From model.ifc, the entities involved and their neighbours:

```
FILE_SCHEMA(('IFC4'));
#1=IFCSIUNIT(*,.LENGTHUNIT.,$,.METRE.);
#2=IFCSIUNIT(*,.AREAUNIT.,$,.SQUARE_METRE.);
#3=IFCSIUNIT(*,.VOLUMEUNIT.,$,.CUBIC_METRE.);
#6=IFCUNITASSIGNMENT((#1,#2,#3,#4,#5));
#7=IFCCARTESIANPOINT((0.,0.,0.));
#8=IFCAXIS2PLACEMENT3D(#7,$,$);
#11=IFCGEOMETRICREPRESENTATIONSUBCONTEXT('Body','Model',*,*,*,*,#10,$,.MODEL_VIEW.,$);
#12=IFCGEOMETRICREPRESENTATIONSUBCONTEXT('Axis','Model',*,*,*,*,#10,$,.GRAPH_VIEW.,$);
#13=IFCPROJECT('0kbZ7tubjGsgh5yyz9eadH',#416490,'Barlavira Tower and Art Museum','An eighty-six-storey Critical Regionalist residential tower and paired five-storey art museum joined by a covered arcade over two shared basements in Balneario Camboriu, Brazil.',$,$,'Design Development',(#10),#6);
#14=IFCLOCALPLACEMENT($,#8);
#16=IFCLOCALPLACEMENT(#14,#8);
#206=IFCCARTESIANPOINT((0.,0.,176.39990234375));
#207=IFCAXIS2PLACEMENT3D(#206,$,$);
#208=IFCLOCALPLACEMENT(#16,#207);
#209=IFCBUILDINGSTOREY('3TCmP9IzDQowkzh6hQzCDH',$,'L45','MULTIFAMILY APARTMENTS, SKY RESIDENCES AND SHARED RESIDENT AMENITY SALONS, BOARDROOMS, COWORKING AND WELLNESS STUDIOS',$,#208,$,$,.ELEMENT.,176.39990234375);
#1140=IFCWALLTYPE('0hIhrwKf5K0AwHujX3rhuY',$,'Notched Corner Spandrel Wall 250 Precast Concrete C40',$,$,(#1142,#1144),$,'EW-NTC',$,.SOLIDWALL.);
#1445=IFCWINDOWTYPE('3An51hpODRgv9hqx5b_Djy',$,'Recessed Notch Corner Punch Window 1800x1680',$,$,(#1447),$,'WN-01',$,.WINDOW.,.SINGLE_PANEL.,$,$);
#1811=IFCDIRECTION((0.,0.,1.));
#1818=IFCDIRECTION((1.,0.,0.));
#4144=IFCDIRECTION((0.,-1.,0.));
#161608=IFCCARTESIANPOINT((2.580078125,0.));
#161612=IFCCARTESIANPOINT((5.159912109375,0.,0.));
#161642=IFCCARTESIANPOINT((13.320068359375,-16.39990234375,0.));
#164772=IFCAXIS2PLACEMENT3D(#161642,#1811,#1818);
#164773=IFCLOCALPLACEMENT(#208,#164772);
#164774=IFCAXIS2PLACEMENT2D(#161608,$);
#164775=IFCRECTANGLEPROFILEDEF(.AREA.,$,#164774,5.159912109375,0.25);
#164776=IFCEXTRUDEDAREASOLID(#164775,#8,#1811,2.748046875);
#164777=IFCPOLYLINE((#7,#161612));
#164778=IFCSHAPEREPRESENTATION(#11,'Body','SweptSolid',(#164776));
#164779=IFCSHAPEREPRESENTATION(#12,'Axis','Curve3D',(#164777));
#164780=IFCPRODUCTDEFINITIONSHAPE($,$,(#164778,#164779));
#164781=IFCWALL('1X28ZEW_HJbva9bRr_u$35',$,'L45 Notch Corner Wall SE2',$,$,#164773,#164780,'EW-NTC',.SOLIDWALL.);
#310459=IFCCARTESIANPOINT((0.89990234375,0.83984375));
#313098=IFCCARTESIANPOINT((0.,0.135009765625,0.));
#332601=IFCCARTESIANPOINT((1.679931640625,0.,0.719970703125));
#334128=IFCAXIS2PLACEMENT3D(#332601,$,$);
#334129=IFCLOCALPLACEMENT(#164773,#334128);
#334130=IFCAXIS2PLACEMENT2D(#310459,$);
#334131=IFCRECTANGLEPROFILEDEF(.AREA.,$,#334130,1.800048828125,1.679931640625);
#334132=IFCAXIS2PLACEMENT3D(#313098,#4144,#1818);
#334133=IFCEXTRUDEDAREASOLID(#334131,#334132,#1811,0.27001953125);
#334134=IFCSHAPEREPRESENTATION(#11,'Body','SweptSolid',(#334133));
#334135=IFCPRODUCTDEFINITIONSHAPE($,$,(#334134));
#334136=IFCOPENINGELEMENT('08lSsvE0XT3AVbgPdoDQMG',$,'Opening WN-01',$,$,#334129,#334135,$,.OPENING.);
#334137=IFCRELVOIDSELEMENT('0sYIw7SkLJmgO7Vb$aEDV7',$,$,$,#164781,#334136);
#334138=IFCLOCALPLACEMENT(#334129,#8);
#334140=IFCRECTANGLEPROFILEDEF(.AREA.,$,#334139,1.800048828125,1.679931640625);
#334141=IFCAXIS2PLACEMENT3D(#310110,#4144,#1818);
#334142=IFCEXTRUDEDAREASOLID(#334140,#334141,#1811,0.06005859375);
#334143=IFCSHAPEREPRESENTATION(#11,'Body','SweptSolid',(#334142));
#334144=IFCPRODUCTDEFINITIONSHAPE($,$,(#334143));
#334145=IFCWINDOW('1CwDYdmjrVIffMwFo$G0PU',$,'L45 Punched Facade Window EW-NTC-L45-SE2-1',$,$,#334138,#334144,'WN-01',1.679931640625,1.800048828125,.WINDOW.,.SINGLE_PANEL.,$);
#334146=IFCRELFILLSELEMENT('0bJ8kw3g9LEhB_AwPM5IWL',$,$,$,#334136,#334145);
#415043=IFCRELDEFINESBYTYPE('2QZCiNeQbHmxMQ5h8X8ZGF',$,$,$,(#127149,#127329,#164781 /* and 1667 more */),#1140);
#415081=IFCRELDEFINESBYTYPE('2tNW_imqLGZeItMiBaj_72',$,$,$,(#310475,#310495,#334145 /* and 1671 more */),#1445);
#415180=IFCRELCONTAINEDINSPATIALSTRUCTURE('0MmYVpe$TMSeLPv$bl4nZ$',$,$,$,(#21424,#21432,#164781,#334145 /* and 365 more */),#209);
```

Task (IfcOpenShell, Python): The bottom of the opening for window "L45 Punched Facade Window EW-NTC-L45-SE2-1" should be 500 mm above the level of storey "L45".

```python
import numpy as np
import ifcopenshell
import ifcopenshell.api.geometry
import ifcopenshell.geom
import ifcopenshell.util.element
import ifcopenshell.util.placement
import ifcopenshell.util.shape
import ifcopenshell.util.unit

model = ifcopenshell.open("model.ifc")
unit_scale = ifcopenshell.util.unit.calculate_unit_scale(model)

window = model.by_guid("1CwDYdmjrVIffMwFo$G0PU")
opening = window.FillsVoids[0].RelatingOpeningElement
storey = ifcopenshell.util.element.get_container(window, ifc_class="IfcBuildingStorey")
level = ifcopenshell.util.placement.get_local_placement(storey.ObjectPlacement)[2, 3]

# The opening's origin need not be at the sill, so measure its lowest point.
shape = ifcopenshell.geom.create_shape(ifcopenshell.geom.settings(), opening)
bottom = ifcopenshell.util.shape.get_shape_bottom_elevation(shape, shape.geometry) / unit_scale
dz = level + 0.5 / unit_scale - bottom

shift = np.array([0.0, 0.0, dz])
# The window is placed relative to its opening, so it follows when the opening moves.
matrix = ifcopenshell.util.placement.get_local_placement(opening.ObjectPlacement)
matrix[:3, 3] += shift
ifcopenshell.api.geometry.edit_object_placement(
    model, product=opening, matrix=matrix, is_si=False, should_transform_children=True
)

print(f"moved by {dz * unit_scale:+.3f} m")

model.write("model-out.ifc")
```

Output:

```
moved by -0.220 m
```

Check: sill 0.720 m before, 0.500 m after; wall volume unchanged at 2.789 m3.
